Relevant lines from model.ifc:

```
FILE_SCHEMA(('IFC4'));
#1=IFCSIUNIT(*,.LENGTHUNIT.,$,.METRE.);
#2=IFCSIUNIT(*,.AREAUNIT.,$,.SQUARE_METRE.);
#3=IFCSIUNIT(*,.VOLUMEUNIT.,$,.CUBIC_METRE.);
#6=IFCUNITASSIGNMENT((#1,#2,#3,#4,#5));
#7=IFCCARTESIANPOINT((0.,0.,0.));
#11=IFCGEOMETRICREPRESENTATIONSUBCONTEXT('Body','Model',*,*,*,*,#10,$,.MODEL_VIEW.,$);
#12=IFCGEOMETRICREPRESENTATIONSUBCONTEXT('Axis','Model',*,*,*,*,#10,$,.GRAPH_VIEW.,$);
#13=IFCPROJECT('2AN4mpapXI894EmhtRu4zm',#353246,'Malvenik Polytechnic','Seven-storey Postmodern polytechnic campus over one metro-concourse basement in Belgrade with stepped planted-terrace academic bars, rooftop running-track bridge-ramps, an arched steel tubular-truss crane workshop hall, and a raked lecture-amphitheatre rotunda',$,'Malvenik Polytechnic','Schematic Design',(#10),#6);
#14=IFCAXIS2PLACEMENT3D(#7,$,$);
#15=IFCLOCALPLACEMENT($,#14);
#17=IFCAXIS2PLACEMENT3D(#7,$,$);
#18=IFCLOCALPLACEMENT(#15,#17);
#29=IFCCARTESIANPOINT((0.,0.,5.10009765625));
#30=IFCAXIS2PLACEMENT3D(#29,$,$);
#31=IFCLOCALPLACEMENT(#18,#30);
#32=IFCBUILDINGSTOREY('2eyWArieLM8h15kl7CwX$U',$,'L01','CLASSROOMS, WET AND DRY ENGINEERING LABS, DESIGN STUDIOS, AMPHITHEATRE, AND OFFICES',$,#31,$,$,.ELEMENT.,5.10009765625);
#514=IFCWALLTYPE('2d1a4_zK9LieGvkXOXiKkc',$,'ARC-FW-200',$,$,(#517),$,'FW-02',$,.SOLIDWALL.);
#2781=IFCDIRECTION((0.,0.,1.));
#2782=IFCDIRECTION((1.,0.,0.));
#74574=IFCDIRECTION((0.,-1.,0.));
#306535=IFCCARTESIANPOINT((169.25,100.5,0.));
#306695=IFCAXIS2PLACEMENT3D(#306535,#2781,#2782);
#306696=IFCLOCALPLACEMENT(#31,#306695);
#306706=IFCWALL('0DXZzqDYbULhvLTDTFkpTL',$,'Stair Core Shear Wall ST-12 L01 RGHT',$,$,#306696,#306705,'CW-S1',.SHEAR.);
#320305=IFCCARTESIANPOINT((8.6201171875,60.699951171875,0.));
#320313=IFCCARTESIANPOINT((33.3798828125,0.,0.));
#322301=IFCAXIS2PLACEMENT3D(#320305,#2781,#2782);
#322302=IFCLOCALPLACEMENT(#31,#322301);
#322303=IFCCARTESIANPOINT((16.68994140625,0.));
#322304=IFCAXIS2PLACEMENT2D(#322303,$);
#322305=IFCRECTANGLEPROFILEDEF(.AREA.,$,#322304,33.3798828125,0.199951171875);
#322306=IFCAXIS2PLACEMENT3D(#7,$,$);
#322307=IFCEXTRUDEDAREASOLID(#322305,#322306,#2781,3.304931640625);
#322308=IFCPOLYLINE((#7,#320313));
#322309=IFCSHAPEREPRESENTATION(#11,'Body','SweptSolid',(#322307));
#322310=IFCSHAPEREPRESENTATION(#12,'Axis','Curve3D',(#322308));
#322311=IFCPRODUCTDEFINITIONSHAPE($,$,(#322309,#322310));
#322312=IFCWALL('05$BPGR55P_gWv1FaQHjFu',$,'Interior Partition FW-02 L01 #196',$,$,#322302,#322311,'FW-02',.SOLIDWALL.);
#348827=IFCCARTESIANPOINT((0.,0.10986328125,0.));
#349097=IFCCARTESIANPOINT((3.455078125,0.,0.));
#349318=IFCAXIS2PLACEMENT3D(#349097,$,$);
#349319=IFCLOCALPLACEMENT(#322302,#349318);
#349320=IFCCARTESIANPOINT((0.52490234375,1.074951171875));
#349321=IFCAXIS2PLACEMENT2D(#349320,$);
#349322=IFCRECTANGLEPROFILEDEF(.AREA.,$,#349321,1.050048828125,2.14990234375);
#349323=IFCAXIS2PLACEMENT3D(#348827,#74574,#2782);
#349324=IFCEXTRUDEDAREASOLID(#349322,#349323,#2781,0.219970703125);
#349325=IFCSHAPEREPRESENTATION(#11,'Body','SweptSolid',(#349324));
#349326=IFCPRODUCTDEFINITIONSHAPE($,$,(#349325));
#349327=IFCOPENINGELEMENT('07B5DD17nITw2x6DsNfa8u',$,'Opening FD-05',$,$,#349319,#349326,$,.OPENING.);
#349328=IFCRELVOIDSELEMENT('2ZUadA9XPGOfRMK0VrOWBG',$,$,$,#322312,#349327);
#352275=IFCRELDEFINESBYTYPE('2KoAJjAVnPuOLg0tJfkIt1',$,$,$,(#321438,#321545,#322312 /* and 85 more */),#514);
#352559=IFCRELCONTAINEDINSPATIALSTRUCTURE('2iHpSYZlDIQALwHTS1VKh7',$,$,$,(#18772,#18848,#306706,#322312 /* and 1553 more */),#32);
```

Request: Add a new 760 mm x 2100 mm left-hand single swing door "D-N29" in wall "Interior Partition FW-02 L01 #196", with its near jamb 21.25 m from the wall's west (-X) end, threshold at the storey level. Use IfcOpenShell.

```python
import numpy as np
import ifcopenshell
import ifcopenshell.api.feature
import ifcopenshell.api.geometry
import ifcopenshell.api.root
import ifcopenshell.api.spatial
import ifcopenshell.geom
import ifcopenshell.util.element
import ifcopenshell.util.placement
import ifcopenshell.util.representation
import ifcopenshell.util.shape
import ifcopenshell.util.unit

model = ifcopenshell.open("model.ifc")
unit_scale = ifcopenshell.util.unit.calculate_unit_scale(model)
settings = ifcopenshell.geom.settings()


def volume(element):
    """Net volume in cubic metres, openings subtracted."""
    shape = ifcopenshell.geom.create_shape(settings, element)
    return ifcopenshell.util.shape.get_volume(shape.geometry)


wall = model.by_guid("05$BPGR55P_gWv1FaQHjFu")
storey = ifcopenshell.util.element.get_container(wall, ifc_class="IfcBuildingStorey")
context = ifcopenshell.util.representation.get_context(model, "Model", "Body", "MODEL_VIEW")
before = volume(wall)

width, height, from_end, sill = 0.76, 2.1, 21.25, 0.0  # metres

# The wall runs along its own X axis, and the end named is its -X end.
wall_shape = ifcopenshell.geom.create_shape(settings, wall)
x, y, z = ifcopenshell.util.shape.get_vertices(wall_shape.geometry).T
start = x.min() + from_end
face, thickness = float(y.min()), float(y.max() - y.min())
wall_matrix = ifcopenshell.util.placement.get_local_placement(wall.ObjectPlacement)
level = ifcopenshell.util.placement.get_local_placement(storey.ObjectPlacement)[2, 3]


def in_wall(x, y):
    """Placement at x, y metres in the wall's axes, at sill height."""
    matrix = wall_matrix.copy()
    matrix[:, 3] = wall_matrix @ np.array([x / unit_scale, y / unit_scale, 0.0, 1.0])
    matrix[2, 3] = level + sill / unit_scale
    return matrix


# Opening: a box that overshoots both wall faces by 50 mm.
opening = ifcopenshell.api.root.create_entity(model, ifc_class="IfcOpeningElement", predefined_type="OPENING")
box = ifcopenshell.api.geometry.add_wall_representation(
    model, context=context, length=width, height=height, thickness=thickness + 0.1
)
ifcopenshell.api.geometry.assign_representation(model, product=opening, representation=box)
ifcopenshell.api.geometry.edit_object_placement(model, product=opening, matrix=in_wall(start, face - 0.05), is_si=False)
ifcopenshell.api.feature.add_feature(model, feature=opening, element=wall)

door = ifcopenshell.api.root.create_entity(model, ifc_class="IfcDoor", name="D-N29", predefined_type="DOOR")
door.OverallWidth, door.OverallHeight = width / unit_scale, height / unit_scale
door.OperationType = "SINGLE_SWING_LEFT"
body = ifcopenshell.api.geometry.add_door_representation(
    model,
    context=context,
    overall_width=door.OverallWidth,
    overall_height=door.OverallHeight,
    operation_type="SINGLE_SWING_LEFT",
    lining_properties={"LiningDepth": thickness / unit_scale, "ThresholdDepth": thickness / unit_scale},
)
ifcopenshell.api.geometry.assign_representation(model, product=door, representation=body)
ifcopenshell.api.spatial.assign_container(model, products=[door], relating_structure=storey)
ifcopenshell.api.feature.add_filling(model, opening=opening, element=door)

# The lining spans the wall, so the door starts at the wall face.
ifcopenshell.api.geometry.edit_object_placement(model, product=door, matrix=in_wall(start, face), is_si=False)

after = volume(wall)

print(f"wall volume {before:.3f} -> {after:.3f} m3")

model.write("model_edited.ifc")
```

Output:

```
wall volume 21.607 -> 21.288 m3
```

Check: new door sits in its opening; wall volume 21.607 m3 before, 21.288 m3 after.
